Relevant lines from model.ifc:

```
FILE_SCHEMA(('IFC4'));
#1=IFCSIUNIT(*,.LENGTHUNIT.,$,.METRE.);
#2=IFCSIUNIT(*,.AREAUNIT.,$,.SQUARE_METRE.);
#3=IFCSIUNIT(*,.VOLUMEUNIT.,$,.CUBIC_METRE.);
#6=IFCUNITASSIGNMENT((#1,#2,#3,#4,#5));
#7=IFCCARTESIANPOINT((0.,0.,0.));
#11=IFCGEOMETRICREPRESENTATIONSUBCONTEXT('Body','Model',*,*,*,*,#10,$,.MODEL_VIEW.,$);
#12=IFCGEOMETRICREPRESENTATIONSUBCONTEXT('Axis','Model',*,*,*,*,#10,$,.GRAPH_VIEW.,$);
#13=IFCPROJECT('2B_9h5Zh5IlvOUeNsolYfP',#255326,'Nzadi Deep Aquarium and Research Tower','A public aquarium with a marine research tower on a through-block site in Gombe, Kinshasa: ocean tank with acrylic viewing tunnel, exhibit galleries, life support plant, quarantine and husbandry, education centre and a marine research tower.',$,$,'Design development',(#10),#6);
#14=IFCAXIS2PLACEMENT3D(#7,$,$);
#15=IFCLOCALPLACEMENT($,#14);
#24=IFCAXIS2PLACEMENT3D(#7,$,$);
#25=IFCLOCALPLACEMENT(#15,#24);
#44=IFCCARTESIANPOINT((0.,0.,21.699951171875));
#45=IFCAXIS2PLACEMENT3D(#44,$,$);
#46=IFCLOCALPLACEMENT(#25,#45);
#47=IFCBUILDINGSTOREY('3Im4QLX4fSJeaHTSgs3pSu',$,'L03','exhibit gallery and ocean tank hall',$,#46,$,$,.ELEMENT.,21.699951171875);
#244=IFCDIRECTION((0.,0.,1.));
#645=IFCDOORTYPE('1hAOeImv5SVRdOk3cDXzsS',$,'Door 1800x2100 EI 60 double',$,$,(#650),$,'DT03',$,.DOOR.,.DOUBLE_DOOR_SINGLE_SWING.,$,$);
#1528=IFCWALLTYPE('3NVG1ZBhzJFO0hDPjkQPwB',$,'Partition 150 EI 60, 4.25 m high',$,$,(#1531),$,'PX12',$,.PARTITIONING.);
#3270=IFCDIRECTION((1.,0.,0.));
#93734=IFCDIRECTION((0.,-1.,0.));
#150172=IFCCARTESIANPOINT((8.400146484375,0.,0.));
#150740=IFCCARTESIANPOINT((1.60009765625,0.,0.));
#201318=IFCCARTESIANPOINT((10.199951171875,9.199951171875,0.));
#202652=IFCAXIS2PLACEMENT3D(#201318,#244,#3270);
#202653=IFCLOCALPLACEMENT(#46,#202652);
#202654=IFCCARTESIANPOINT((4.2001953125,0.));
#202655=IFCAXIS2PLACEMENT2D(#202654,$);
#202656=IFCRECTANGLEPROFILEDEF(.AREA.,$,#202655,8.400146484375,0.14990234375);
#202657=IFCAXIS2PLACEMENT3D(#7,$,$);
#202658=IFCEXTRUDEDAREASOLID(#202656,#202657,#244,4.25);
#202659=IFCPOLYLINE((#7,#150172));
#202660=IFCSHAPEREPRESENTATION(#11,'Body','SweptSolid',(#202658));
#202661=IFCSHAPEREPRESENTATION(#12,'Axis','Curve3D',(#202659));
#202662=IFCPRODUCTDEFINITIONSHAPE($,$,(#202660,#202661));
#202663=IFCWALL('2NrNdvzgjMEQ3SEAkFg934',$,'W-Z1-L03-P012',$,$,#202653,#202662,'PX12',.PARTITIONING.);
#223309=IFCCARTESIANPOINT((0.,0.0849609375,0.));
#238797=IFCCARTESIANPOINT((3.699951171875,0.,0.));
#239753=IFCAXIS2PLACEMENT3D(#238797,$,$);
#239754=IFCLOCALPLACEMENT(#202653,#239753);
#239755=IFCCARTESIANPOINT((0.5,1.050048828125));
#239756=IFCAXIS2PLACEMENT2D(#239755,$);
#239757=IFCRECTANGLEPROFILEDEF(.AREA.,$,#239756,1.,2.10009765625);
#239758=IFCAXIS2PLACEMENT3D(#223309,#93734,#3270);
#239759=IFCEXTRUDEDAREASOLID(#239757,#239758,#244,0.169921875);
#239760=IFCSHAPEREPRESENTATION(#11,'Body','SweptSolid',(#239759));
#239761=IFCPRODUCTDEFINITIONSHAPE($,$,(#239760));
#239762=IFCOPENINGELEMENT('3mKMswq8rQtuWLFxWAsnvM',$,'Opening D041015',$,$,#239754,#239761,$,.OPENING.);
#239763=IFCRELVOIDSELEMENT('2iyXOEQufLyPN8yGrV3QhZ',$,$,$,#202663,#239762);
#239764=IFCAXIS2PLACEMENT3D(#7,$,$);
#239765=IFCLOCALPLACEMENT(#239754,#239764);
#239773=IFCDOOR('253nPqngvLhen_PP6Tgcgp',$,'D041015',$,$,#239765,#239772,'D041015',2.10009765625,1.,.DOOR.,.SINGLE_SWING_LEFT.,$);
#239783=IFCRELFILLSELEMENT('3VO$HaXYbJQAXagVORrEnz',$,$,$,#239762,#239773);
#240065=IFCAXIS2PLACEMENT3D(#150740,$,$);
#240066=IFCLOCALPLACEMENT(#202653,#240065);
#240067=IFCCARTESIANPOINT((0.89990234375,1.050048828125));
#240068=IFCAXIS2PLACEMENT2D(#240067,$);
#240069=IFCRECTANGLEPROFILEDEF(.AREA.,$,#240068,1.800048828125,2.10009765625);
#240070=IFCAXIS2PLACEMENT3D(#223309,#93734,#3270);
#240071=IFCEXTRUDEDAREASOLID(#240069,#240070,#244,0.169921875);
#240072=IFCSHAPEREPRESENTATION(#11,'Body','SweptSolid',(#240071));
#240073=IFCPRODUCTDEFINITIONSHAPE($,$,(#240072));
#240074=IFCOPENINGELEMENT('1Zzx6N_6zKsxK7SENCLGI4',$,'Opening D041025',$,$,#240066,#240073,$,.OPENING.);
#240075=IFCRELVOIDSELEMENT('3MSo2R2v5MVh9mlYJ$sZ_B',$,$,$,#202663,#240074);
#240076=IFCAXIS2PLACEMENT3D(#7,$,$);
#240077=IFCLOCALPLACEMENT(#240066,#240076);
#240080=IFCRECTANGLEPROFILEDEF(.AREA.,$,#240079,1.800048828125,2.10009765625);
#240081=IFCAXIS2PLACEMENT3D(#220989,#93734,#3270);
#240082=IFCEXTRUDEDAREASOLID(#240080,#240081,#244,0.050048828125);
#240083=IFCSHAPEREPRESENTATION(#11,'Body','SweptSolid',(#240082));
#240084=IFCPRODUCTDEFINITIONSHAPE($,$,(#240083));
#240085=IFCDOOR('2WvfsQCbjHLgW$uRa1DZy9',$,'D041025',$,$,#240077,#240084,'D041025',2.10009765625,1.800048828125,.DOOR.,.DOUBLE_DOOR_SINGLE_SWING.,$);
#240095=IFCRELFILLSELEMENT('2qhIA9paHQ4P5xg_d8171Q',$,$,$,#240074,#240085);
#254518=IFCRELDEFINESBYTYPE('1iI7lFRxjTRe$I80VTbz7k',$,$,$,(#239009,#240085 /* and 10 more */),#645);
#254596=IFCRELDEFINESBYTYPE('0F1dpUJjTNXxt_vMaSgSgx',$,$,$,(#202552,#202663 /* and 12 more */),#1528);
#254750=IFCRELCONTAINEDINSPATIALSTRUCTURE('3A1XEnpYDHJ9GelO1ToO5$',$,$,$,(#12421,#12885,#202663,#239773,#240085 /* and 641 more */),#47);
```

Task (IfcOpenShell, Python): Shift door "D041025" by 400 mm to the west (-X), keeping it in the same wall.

```python
import ifcopenshell
import ifcopenshell.api.geometry
import ifcopenshell.util.placement

model = ifcopenshell.open("model.ifc")

door = model.by_guid("2WvfsQCbjHLgW$uRa1DZy9")
opening = door.FillsVoids[0].RelatingOpeningElement
wall = opening.VoidsElements[0].RelatingBuildingElement

wall_matrix = ifcopenshell.util.placement.get_local_placement(wall.ObjectPlacement)
shift = wall_matrix[:3, 0] * -0.4
before = ifcopenshell.util.placement.get_local_placement(door.ObjectPlacement)[:3, 3].copy()

# The door is placed relative to its opening, so it follows when the opening moves.
matrix = ifcopenshell.util.placement.get_local_placement(opening.ObjectPlacement)
matrix[:3, 3] += shift
ifcopenshell.api.geometry.edit_object_placement(
    model, product=opening, matrix=matrix, is_si=False, should_transform_children=True
)

after = ifcopenshell.util.placement.get_local_placement(door.ObjectPlacement)[:3, 3]
print("door moved by", (after - before).round(3) + 0.0)

model.write("model_edited.ifc")
```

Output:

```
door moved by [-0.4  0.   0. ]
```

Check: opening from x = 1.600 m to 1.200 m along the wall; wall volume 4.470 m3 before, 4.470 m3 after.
